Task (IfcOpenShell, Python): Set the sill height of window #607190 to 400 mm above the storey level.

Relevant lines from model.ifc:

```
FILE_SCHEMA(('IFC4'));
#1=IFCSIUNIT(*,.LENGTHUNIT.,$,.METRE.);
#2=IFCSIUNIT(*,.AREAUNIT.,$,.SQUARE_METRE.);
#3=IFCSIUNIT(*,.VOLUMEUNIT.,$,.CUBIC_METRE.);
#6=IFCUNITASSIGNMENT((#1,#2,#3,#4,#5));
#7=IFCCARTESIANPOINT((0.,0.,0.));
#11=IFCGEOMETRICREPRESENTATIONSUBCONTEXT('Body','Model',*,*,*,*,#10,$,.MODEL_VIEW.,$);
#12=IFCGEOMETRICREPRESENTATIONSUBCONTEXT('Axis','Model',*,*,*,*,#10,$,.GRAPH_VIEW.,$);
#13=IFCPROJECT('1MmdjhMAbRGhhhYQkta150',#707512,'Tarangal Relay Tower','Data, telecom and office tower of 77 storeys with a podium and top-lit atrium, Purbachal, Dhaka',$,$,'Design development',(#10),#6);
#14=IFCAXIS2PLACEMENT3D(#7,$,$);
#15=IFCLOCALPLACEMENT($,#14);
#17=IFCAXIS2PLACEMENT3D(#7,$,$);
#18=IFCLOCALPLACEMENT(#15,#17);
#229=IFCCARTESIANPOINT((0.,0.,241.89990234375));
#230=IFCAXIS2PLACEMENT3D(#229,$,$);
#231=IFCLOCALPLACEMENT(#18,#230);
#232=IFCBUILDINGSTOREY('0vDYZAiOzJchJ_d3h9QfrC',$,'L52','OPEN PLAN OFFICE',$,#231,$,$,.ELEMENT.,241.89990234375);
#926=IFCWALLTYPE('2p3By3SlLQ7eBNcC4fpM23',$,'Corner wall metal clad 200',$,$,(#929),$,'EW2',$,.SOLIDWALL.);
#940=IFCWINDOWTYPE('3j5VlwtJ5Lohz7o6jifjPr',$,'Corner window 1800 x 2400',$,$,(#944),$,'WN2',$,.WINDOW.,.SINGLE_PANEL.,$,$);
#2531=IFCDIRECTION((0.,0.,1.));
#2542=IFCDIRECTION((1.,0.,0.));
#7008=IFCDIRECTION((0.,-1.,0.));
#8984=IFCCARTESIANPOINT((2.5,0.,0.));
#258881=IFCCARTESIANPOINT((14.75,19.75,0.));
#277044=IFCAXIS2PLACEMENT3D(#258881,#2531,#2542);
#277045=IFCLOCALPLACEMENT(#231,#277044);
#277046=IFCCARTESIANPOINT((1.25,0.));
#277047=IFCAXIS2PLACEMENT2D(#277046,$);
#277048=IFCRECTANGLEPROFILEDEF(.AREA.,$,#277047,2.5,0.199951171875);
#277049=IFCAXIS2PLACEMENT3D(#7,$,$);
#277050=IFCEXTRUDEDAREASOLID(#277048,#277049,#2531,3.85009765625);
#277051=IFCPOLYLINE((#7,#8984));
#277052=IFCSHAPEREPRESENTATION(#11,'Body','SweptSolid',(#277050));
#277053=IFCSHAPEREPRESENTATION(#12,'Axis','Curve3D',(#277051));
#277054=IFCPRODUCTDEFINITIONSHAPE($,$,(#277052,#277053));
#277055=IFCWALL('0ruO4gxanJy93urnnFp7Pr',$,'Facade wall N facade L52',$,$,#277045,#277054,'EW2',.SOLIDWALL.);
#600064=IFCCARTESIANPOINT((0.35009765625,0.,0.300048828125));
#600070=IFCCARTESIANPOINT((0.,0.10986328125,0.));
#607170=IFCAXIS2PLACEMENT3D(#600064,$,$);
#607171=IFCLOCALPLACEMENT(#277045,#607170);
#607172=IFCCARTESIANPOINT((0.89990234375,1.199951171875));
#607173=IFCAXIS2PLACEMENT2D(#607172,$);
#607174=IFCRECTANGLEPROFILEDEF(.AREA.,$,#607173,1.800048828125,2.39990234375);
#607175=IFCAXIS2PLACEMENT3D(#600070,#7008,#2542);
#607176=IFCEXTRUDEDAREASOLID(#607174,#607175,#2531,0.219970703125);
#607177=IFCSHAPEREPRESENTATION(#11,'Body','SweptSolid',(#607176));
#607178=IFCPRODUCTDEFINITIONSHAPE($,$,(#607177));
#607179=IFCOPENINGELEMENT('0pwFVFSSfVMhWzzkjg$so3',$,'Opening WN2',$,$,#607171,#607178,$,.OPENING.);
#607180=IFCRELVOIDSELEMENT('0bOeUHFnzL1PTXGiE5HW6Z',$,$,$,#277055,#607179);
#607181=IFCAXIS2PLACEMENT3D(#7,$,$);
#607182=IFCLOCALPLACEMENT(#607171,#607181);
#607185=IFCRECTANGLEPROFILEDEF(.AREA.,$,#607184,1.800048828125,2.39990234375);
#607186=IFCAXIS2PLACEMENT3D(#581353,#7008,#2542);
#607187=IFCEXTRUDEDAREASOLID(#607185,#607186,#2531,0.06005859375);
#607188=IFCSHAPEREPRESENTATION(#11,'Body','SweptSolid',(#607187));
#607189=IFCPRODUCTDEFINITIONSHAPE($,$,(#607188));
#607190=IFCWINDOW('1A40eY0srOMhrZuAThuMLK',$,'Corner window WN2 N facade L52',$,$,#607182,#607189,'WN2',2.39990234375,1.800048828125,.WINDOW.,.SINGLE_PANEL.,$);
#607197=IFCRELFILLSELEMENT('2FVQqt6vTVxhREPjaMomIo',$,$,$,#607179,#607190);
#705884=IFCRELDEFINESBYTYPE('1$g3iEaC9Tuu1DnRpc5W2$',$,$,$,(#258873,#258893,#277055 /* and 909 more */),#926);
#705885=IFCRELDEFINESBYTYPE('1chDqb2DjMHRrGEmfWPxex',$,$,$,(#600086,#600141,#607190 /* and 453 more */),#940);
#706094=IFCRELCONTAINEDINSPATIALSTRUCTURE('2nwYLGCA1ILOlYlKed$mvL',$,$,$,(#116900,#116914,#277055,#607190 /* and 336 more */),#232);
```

```python
import numpy as np
import ifcopenshell
import ifcopenshell.api.geometry
import ifcopenshell.geom
import ifcopenshell.util.element
import ifcopenshell.util.placement
import ifcopenshell.util.shape
import ifcopenshell.util.unit

model = ifcopenshell.open("model.ifc")
unit_scale = ifcopenshell.util.unit.calculate_unit_scale(model)

window = model.by_guid("1A40eY0srOMhrZuAThuMLK")
opening = window.FillsVoids[0].RelatingOpeningElement
storey = ifcopenshell.util.element.get_container(window, ifc_class="IfcBuildingStorey")
level = ifcopenshell.util.placement.get_local_placement(storey.ObjectPlacement)[2, 3]

# The opening's origin need not be at the sill, so measure its lowest point.
shape = ifcopenshell.geom.create_shape(ifcopenshell.geom.settings(), opening)
bottom = ifcopenshell.util.shape.get_shape_bottom_elevation(shape, shape.geometry) / unit_scale
dz = level + 0.4 / unit_scale - bottom

shift = np.array([0.0, 0.0, dz])
# The window is placed relative to its opening, so it follows when the opening moves.
matrix = ifcopenshell.util.placement.get_local_placement(opening.ObjectPlacement)
matrix[:3, 3] += shift
ifcopenshell.api.geometry.edit_object_placement(
    model, product=opening, matrix=matrix, is_si=False, should_transform_children=True
)

print(f"moved by {dz * unit_scale:+.3f} m")

model.write("model_v2.ifc")
```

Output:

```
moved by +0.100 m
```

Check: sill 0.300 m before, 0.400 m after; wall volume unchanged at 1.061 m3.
